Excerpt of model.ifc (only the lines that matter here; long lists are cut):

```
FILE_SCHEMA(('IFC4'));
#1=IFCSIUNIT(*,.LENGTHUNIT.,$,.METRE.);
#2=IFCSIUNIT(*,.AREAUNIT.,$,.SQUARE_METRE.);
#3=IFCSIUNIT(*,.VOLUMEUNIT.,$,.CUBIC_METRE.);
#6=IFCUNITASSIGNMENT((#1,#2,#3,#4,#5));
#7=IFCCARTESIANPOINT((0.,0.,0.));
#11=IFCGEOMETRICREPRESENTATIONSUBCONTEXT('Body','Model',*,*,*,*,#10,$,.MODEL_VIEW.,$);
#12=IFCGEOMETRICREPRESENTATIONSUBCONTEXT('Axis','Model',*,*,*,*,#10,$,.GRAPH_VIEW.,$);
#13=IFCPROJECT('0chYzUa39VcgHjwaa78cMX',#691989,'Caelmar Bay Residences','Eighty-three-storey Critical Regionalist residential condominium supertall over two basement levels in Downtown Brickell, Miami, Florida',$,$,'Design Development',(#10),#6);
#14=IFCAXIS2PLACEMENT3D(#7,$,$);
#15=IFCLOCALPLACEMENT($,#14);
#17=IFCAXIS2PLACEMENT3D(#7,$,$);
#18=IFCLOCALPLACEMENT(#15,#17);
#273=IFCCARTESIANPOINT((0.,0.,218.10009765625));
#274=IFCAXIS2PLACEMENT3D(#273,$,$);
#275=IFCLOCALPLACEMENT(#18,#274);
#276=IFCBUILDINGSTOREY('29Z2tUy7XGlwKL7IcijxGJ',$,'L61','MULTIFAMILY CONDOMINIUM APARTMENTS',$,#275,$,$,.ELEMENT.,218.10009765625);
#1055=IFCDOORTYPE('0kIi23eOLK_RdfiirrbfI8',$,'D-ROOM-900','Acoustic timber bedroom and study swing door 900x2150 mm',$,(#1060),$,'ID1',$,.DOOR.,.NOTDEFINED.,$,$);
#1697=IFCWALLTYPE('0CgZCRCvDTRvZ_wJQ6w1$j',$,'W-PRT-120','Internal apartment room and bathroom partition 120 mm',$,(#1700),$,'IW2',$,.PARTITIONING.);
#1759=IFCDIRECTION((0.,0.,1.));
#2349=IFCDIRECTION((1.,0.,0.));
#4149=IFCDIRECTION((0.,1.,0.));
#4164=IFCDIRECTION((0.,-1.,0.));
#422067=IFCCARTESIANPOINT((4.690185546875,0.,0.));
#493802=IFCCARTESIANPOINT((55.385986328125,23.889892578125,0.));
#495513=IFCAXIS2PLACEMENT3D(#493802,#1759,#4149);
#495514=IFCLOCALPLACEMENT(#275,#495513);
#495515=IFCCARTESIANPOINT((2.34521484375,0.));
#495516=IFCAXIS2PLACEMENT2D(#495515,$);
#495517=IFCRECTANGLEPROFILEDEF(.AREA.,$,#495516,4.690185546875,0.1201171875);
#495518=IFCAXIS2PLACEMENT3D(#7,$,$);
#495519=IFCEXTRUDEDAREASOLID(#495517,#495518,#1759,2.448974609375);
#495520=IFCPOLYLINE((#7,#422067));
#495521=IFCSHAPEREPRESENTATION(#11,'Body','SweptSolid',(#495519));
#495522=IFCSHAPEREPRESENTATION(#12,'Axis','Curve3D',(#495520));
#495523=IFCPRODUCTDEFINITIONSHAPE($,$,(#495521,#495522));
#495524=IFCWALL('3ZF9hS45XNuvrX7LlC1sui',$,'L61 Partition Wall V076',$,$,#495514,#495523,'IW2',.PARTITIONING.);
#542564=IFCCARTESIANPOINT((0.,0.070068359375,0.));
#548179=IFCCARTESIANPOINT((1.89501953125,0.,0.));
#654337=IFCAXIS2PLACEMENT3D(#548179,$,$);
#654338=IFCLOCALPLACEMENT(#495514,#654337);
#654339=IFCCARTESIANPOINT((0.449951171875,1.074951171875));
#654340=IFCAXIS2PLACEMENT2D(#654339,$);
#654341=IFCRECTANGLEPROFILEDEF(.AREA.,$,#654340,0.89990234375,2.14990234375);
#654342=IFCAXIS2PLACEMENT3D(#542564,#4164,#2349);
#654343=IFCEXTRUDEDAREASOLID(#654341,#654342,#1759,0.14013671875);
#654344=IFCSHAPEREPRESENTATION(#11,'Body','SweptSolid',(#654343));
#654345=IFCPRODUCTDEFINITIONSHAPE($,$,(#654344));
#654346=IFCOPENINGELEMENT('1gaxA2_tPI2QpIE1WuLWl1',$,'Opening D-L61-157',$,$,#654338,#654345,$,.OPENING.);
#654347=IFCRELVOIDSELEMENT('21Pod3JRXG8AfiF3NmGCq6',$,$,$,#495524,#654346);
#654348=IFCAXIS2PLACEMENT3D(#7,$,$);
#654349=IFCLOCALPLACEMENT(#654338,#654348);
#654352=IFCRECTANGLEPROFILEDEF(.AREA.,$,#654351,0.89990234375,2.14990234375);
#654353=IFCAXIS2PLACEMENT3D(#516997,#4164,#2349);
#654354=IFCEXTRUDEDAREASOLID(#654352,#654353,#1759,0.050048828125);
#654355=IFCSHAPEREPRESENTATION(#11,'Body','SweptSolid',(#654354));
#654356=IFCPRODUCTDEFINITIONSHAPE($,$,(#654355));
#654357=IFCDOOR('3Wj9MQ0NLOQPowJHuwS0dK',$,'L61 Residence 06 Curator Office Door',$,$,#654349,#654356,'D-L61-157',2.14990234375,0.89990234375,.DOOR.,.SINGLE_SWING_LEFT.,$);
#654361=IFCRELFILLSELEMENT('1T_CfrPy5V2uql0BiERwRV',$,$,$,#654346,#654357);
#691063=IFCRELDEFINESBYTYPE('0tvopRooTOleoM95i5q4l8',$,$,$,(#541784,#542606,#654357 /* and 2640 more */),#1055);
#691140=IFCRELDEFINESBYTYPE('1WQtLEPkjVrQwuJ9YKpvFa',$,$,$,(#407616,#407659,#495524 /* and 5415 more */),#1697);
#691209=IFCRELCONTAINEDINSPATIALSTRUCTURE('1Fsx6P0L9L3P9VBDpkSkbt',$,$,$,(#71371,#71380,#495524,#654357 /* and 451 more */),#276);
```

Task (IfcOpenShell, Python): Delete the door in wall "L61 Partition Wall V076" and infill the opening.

```python
import ifcopenshell
import ifcopenshell.api.feature
import ifcopenshell.api.root
import ifcopenshell.geom
import ifcopenshell.util.shape

model = ifcopenshell.open("model.ifc")
settings = ifcopenshell.geom.settings()


def volume(element):
    """Net volume in cubic metres, openings subtracted."""
    shape = ifcopenshell.geom.create_shape(settings, element)
    return ifcopenshell.util.shape.get_volume(shape.geometry)


door = model.by_guid("3Wj9MQ0NLOQPowJHuwS0dK")
opening = door.FillsVoids[0].RelatingOpeningElement
wall = opening.VoidsElements[0].RelatingBuildingElement
before = volume(wall)

ifcopenshell.api.root.remove_product(model, product=door)
ifcopenshell.api.feature.remove_feature(model, feature=opening)

after = volume(wall)

print(f"wall volume {before:.3f} -> {after:.3f} m3")

model.write("model_edited.ifc")
```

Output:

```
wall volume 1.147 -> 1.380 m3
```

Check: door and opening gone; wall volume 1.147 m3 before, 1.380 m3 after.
